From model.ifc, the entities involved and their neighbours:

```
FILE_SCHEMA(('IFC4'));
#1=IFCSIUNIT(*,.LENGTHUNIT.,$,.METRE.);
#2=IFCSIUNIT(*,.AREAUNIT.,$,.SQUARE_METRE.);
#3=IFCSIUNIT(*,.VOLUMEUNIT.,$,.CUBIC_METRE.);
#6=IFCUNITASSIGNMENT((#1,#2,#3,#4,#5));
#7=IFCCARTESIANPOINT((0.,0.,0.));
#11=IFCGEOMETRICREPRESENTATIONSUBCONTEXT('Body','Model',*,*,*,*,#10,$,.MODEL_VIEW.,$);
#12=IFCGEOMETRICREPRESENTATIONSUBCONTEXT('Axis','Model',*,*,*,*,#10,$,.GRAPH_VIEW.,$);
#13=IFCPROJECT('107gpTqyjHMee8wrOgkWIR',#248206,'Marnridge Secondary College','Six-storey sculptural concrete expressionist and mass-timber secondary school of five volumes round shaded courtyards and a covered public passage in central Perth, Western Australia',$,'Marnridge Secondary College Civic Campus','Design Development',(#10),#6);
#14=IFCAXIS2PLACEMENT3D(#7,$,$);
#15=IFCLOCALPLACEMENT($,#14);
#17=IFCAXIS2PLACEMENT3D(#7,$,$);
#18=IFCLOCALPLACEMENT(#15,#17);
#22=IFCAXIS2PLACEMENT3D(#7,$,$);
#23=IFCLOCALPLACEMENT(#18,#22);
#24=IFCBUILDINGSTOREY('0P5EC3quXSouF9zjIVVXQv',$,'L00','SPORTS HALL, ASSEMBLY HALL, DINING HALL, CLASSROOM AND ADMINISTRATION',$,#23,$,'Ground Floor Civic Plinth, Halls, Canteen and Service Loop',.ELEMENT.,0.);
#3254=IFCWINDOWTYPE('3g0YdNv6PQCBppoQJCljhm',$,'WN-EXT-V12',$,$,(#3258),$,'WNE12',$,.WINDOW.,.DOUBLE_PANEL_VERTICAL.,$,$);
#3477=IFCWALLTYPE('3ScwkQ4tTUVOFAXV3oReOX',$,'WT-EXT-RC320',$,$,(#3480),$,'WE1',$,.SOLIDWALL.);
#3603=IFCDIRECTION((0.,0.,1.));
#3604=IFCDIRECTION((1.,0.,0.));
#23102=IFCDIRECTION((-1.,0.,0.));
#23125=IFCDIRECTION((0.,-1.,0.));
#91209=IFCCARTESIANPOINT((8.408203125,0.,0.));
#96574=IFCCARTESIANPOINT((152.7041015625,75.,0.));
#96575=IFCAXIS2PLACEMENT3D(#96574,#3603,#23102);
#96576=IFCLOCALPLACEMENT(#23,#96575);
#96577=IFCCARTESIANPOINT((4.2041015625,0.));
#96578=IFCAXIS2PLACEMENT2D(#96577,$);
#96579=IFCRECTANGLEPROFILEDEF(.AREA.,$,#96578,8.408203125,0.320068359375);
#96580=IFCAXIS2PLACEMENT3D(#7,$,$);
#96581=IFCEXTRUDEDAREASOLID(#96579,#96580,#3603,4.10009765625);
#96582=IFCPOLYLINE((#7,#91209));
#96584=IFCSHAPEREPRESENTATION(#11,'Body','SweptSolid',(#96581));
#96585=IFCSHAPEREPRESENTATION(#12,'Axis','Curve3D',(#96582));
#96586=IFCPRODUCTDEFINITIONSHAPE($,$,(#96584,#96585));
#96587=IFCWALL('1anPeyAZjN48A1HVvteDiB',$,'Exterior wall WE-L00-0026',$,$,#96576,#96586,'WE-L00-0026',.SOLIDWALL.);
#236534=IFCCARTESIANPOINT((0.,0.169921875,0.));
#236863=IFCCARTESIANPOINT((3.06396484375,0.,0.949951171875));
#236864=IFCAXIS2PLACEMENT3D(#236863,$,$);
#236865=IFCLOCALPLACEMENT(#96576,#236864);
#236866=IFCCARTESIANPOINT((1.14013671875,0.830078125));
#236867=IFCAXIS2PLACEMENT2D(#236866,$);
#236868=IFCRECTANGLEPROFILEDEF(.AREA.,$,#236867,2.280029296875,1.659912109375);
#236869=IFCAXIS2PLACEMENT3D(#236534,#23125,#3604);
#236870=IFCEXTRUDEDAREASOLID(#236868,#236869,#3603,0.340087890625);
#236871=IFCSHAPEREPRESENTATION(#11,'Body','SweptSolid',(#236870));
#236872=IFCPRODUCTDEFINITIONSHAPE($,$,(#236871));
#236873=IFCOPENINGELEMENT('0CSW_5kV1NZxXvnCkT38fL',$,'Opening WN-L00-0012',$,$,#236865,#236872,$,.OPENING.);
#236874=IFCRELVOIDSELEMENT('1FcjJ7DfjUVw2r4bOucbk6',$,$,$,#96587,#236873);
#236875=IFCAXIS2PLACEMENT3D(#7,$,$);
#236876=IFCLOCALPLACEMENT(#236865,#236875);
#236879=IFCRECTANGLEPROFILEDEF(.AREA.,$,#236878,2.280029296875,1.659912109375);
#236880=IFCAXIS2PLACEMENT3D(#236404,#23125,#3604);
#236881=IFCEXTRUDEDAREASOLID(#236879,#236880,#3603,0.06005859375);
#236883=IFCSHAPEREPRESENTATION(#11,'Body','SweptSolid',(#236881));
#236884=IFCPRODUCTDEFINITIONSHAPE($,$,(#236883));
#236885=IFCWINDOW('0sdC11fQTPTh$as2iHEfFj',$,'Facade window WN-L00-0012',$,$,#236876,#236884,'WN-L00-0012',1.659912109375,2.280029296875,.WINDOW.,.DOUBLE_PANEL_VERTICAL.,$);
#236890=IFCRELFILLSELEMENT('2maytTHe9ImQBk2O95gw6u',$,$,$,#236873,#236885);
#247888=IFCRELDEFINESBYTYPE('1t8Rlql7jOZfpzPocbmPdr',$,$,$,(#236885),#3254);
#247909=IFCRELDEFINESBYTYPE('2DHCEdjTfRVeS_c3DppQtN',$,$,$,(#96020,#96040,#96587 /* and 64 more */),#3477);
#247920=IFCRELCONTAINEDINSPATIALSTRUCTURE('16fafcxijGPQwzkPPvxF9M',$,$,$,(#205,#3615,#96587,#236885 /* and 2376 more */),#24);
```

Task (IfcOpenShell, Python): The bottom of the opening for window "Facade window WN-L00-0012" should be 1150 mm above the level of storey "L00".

```python
import numpy as np
import ifcopenshell
import ifcopenshell.api.geometry
import ifcopenshell.geom
import ifcopenshell.util.element
import ifcopenshell.util.placement
import ifcopenshell.util.shape
import ifcopenshell.util.unit

model = ifcopenshell.open("model.ifc")
unit_scale = ifcopenshell.util.unit.calculate_unit_scale(model)

window = model.by_guid("0sdC11fQTPTh$as2iHEfFj")
opening = window.FillsVoids[0].RelatingOpeningElement
storey = ifcopenshell.util.element.get_container(window, ifc_class="IfcBuildingStorey")
level = ifcopenshell.util.placement.get_local_placement(storey.ObjectPlacement)[2, 3]

# The opening's origin need not be at the sill, so measure its lowest point.
shape = ifcopenshell.geom.create_shape(ifcopenshell.geom.settings(), opening)
bottom = ifcopenshell.util.shape.get_shape_bottom_elevation(shape, shape.geometry) / unit_scale
dz = level + 1.15 / unit_scale - bottom

shift = np.array([0.0, 0.0, dz])
# The window is placed relative to its opening, so it follows when the opening moves.
matrix = ifcopenshell.util.placement.get_local_placement(opening.ObjectPlacement)
matrix[:3, 3] += shift
ifcopenshell.api.geometry.edit_object_placement(
    model, product=opening, matrix=matrix, is_si=False, should_transform_children=True
)

print(f"moved by {dz * unit_scale:+.3f} m")

model.write("model_edited.ifc")
```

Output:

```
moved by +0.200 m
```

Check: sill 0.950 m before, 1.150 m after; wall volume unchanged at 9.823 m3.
